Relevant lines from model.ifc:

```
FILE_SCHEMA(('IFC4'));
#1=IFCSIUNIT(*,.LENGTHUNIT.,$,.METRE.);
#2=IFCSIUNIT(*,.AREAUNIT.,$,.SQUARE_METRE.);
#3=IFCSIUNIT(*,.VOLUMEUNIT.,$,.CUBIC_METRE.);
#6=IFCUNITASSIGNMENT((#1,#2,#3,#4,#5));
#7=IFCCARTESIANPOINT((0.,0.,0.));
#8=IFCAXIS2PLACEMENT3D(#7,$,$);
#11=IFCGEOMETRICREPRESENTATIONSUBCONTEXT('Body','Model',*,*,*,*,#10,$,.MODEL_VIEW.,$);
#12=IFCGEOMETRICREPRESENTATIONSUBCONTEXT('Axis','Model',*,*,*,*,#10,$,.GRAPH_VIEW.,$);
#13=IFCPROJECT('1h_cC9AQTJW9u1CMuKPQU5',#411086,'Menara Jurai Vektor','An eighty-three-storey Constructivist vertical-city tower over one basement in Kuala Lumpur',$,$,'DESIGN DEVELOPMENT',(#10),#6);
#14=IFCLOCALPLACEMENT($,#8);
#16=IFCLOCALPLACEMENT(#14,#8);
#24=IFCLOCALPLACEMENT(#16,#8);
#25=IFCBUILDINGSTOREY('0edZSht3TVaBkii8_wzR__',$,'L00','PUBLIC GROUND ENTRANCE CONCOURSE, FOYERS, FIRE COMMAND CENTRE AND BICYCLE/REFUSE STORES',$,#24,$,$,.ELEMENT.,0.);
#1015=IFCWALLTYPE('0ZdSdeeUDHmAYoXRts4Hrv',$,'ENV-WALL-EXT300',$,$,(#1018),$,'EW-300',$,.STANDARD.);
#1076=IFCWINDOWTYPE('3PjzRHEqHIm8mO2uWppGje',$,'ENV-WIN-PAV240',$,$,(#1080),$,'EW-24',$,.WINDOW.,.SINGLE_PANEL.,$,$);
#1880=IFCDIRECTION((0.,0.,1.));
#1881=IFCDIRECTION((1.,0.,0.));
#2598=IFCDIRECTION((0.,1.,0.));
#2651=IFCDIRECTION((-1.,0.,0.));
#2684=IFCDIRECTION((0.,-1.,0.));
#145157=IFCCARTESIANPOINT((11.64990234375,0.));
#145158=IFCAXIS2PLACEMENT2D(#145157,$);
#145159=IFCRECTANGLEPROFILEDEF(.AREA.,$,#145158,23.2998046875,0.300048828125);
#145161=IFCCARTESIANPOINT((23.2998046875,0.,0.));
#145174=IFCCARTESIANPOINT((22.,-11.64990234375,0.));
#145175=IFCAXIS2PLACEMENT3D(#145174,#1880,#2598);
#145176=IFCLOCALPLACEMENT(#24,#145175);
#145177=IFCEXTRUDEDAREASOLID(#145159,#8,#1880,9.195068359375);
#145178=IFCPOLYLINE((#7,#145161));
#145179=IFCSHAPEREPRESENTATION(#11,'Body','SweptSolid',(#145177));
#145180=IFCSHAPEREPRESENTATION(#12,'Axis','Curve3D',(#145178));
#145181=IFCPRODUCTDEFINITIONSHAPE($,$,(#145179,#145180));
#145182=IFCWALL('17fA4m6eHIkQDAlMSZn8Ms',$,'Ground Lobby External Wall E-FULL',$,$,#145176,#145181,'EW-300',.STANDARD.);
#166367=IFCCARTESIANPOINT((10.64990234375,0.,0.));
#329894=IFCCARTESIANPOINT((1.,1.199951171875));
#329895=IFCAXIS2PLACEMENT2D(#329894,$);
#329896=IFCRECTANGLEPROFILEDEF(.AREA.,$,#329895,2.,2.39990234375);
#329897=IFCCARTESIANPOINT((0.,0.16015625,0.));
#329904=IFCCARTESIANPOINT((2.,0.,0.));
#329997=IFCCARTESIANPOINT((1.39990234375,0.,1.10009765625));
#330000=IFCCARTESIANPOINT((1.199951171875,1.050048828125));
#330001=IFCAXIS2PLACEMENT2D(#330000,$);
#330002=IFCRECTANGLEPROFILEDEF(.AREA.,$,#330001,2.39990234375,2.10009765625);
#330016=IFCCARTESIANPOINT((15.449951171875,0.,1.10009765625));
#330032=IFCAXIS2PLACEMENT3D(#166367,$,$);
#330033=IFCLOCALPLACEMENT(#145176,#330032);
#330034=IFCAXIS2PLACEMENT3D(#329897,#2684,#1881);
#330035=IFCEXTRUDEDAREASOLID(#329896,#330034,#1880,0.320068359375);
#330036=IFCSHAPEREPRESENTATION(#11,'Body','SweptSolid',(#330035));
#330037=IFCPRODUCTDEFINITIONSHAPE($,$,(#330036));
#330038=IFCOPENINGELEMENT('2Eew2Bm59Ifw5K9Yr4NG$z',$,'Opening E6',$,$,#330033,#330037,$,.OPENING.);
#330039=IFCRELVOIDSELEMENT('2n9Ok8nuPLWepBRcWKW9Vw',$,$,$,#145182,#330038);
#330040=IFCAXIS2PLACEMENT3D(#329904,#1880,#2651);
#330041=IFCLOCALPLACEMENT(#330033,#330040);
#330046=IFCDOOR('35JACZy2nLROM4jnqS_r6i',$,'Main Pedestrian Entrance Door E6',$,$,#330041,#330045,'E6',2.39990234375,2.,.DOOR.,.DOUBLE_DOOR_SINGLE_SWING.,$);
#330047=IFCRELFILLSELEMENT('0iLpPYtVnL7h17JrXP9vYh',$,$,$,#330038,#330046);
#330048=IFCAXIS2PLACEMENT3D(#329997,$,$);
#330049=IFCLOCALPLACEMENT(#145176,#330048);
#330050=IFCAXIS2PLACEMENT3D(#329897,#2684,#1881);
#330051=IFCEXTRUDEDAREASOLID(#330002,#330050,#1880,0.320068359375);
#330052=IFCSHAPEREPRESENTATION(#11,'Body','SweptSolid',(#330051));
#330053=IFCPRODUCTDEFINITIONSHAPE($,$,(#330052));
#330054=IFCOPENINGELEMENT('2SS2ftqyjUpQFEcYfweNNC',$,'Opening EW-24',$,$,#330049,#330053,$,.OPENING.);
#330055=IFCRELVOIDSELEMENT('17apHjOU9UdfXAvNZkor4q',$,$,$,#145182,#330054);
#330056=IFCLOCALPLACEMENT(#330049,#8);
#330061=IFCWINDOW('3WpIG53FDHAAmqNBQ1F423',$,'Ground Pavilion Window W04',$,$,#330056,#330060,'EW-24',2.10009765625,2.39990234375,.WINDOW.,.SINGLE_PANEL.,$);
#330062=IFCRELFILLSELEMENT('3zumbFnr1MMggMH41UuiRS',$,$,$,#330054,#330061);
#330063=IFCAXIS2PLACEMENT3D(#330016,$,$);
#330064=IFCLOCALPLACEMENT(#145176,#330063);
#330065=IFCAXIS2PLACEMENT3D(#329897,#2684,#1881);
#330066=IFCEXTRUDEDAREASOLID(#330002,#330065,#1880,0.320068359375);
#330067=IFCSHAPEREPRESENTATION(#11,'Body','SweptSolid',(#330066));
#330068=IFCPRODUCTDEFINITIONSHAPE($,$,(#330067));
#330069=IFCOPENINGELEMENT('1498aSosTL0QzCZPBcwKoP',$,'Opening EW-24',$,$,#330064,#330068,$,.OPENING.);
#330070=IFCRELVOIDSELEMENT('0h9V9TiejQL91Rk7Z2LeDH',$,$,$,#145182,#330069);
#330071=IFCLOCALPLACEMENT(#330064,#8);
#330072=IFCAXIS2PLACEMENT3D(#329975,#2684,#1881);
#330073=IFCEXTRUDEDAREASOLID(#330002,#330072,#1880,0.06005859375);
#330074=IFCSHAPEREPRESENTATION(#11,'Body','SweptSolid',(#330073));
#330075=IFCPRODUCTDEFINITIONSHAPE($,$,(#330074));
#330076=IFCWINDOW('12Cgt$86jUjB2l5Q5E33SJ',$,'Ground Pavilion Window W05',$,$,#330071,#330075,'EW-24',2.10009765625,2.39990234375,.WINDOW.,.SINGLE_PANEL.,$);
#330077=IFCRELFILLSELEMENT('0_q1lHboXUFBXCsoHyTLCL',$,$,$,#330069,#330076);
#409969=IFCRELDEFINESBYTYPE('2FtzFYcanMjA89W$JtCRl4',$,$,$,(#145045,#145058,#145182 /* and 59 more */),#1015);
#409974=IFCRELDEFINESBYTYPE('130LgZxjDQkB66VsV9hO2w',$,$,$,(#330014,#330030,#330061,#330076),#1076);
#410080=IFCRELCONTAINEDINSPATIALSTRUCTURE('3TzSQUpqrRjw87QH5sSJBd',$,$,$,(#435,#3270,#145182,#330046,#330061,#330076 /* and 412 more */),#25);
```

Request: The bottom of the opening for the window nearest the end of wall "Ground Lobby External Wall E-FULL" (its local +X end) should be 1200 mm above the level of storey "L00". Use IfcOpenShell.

```python
import numpy as np
import ifcopenshell
import ifcopenshell.api.geometry
import ifcopenshell.geom
import ifcopenshell.util.element
import ifcopenshell.util.placement
import ifcopenshell.util.shape
import ifcopenshell.util.unit

model = ifcopenshell.open("model.ifc")
unit_scale = ifcopenshell.util.unit.calculate_unit_scale(model)

window = model.by_guid("12Cgt$86jUjB2l5Q5E33SJ")
opening = window.FillsVoids[0].RelatingOpeningElement
storey = ifcopenshell.util.element.get_container(window, ifc_class="IfcBuildingStorey")
level = ifcopenshell.util.placement.get_local_placement(storey.ObjectPlacement)[2, 3]

# The opening's origin need not be at the sill, so measure its lowest point.
shape = ifcopenshell.geom.create_shape(ifcopenshell.geom.settings(), opening)
bottom = ifcopenshell.util.shape.get_shape_bottom_elevation(shape, shape.geometry) / unit_scale
dz = level + 1.2 - bottom

shift = np.array([0.0, 0.0, dz])
# The window is placed relative to its opening, so it follows when the opening moves.
matrix = ifcopenshell.util.placement.get_local_placement(opening.ObjectPlacement)
matrix[:3, 3] += shift
ifcopenshell.api.geometry.edit_object_placement(
    model, product=opening, matrix=matrix, is_si=False, should_transform_children=True
)

print(f"moved by {dz * unit_scale:+.3f} m")

model.write("model_updated.ifc")
```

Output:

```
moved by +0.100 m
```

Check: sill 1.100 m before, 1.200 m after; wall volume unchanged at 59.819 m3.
